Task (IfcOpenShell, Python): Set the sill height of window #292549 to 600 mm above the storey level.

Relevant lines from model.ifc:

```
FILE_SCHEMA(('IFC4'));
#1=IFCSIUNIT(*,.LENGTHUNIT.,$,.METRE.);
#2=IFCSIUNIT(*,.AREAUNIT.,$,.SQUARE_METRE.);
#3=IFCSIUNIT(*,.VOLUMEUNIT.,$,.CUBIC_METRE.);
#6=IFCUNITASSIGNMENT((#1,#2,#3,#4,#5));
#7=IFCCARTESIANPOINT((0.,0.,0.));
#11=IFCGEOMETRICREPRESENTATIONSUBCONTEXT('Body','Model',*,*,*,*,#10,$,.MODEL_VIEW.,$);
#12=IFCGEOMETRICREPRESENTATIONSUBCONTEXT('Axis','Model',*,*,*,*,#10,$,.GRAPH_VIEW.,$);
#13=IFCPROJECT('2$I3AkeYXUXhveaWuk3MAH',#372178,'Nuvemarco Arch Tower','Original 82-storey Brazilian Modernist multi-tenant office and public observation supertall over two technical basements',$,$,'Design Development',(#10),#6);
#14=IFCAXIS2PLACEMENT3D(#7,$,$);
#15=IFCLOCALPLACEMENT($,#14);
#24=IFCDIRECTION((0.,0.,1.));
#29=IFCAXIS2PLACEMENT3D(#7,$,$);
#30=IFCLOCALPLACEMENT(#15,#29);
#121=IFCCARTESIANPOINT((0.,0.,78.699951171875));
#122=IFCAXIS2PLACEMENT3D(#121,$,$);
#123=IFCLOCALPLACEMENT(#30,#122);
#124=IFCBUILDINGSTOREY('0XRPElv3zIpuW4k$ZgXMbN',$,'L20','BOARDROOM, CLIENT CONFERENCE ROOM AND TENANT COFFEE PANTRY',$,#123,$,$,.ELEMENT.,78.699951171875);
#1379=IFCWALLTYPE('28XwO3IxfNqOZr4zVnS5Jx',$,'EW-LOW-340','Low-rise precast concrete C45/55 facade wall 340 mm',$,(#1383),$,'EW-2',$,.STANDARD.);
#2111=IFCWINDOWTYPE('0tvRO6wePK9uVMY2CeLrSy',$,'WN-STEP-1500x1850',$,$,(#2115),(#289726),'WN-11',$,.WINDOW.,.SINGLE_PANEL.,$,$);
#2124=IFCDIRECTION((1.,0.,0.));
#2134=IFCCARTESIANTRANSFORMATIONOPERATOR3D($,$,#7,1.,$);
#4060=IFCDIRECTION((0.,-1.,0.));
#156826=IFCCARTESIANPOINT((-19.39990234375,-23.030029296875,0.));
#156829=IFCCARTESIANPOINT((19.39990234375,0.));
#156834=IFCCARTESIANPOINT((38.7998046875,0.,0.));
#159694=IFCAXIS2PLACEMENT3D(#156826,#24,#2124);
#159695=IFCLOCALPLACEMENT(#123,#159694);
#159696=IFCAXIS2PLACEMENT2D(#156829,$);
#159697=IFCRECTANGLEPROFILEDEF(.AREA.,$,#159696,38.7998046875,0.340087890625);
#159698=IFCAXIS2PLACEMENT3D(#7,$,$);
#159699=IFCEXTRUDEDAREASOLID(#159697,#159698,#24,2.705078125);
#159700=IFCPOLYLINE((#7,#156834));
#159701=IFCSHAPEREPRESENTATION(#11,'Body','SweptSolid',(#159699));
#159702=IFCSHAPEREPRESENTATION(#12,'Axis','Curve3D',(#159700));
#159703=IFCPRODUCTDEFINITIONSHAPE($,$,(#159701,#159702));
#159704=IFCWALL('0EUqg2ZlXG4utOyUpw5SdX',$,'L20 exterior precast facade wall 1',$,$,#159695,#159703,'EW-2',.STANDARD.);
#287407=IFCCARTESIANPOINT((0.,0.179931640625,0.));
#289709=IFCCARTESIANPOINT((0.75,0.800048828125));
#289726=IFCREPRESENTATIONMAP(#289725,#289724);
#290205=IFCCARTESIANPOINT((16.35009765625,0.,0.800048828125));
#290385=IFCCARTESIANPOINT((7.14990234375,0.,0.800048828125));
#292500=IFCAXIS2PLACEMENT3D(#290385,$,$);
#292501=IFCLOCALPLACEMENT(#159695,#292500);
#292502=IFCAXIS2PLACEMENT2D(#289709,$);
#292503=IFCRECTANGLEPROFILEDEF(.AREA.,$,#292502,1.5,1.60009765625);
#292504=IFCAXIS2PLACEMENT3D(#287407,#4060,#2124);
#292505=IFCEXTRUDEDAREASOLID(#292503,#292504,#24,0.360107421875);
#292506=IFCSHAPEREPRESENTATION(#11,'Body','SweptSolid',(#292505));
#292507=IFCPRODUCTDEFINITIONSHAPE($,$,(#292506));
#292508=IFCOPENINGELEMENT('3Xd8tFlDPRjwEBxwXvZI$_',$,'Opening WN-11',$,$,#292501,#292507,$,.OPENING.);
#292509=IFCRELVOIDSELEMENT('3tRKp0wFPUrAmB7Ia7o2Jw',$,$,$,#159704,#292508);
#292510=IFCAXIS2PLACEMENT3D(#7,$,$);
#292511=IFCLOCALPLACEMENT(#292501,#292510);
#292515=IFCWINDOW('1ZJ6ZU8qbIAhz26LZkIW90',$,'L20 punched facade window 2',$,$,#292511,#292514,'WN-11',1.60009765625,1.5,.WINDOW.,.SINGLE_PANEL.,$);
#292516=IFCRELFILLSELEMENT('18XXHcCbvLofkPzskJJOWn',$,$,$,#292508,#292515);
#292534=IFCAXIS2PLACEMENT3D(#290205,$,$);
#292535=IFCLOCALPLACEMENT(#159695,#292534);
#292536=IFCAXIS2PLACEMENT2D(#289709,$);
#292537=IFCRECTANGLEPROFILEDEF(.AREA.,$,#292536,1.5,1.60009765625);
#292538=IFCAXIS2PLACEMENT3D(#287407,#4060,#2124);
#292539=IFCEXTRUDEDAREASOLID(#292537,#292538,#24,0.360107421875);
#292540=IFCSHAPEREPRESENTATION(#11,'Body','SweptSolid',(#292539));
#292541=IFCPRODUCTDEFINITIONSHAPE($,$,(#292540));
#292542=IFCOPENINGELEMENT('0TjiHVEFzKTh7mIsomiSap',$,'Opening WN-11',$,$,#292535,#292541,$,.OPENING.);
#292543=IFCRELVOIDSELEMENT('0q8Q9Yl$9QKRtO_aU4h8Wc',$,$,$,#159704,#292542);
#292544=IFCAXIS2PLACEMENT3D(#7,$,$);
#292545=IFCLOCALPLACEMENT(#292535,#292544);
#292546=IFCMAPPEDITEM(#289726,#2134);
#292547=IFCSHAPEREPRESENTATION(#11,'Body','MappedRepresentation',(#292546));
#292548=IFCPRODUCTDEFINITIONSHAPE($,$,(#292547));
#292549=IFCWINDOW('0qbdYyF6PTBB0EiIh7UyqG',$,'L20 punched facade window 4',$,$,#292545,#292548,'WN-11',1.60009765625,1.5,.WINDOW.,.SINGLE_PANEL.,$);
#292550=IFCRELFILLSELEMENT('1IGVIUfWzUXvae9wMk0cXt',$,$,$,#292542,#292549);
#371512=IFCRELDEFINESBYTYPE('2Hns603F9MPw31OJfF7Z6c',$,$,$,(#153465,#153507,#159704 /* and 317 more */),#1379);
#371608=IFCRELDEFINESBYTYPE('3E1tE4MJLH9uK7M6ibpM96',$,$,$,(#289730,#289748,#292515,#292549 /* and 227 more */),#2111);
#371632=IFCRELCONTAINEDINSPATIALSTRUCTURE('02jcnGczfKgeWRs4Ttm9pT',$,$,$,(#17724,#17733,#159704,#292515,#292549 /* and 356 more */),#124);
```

```python
import numpy as np
import ifcopenshell
import ifcopenshell.api.geometry
import ifcopenshell.geom
import ifcopenshell.util.element
import ifcopenshell.util.placement
import ifcopenshell.util.shape
import ifcopenshell.util.unit

model = ifcopenshell.open("model.ifc")
unit_scale = ifcopenshell.util.unit.calculate_unit_scale(model)

window = model.by_guid("0qbdYyF6PTBB0EiIh7UyqG")
opening = window.FillsVoids[0].RelatingOpeningElement
storey = ifcopenshell.util.element.get_container(window, ifc_class="IfcBuildingStorey")
level = ifcopenshell.util.placement.get_local_placement(storey.ObjectPlacement)[2, 3]

# The opening's origin need not be at the sill, so measure its lowest point.
shape = ifcopenshell.geom.create_shape(ifcopenshell.geom.settings(), opening)
bottom = ifcopenshell.util.shape.get_shape_bottom_elevation(shape, shape.geometry) / unit_scale
dz = level + 0.6 - bottom

shift = np.array([0.0, 0.0, dz])
# The window is placed relative to its opening, so it follows when the opening moves.
matrix = ifcopenshell.util.placement.get_local_placement(opening.ObjectPlacement)
matrix[:3, 3] += shift
ifcopenshell.api.geometry.edit_object_placement(
    model, product=opening, matrix=matrix, is_si=False, should_transform_children=True
)

print(f"moved by {dz * unit_scale:+.3f} m")

model.write("model-out.ifc")
```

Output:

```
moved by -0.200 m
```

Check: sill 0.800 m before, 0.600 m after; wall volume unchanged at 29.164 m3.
